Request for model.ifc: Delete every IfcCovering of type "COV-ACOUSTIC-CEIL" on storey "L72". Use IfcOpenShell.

First a look at what the model holds.

```python
import ifcopenshell
import ifcopenshell.util.element

model = ifcopenshell.open("model.ifc")
print(model.schema)
storey = next(s for s in model.by_type("IfcBuildingStorey") if s.Name == "L72")
coverings = [e for e in ifcopenshell.util.element.get_decomposition(storey) if e.is_a("IfcCovering")]
seen = {}
for e in coverings:
    element_type = ifcopenshell.util.element.get_type(e)
    name = element_type.Name if element_type not in (None, e) else None
    seen[name] = seen.get(name, 0) + 1
for name, count in sorted(seen.items(), key=str):
    print(count, "x", name)
```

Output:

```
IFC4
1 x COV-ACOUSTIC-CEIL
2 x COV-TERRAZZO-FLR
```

```python
import ifcopenshell
import ifcopenshell.api.root
import ifcopenshell.util.element

model = ifcopenshell.open("model.ifc")

storey = next(s for s in model.by_type("IfcBuildingStorey") if s.Name == "L72")
coverings = [e for e in ifcopenshell.util.element.get_decomposition(storey) if e.is_a("IfcCovering")]
targets = [e for e in coverings if (t := ifcopenshell.util.element.get_type(e)) not in (None, e) and t.Name == "COV-ACOUSTIC-CEIL"]

for e in targets:
    ifcopenshell.api.root.remove_product(model, product=e)
print(len(targets), "removed")

model.write("model_v2.ifc")
```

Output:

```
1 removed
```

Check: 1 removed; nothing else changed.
